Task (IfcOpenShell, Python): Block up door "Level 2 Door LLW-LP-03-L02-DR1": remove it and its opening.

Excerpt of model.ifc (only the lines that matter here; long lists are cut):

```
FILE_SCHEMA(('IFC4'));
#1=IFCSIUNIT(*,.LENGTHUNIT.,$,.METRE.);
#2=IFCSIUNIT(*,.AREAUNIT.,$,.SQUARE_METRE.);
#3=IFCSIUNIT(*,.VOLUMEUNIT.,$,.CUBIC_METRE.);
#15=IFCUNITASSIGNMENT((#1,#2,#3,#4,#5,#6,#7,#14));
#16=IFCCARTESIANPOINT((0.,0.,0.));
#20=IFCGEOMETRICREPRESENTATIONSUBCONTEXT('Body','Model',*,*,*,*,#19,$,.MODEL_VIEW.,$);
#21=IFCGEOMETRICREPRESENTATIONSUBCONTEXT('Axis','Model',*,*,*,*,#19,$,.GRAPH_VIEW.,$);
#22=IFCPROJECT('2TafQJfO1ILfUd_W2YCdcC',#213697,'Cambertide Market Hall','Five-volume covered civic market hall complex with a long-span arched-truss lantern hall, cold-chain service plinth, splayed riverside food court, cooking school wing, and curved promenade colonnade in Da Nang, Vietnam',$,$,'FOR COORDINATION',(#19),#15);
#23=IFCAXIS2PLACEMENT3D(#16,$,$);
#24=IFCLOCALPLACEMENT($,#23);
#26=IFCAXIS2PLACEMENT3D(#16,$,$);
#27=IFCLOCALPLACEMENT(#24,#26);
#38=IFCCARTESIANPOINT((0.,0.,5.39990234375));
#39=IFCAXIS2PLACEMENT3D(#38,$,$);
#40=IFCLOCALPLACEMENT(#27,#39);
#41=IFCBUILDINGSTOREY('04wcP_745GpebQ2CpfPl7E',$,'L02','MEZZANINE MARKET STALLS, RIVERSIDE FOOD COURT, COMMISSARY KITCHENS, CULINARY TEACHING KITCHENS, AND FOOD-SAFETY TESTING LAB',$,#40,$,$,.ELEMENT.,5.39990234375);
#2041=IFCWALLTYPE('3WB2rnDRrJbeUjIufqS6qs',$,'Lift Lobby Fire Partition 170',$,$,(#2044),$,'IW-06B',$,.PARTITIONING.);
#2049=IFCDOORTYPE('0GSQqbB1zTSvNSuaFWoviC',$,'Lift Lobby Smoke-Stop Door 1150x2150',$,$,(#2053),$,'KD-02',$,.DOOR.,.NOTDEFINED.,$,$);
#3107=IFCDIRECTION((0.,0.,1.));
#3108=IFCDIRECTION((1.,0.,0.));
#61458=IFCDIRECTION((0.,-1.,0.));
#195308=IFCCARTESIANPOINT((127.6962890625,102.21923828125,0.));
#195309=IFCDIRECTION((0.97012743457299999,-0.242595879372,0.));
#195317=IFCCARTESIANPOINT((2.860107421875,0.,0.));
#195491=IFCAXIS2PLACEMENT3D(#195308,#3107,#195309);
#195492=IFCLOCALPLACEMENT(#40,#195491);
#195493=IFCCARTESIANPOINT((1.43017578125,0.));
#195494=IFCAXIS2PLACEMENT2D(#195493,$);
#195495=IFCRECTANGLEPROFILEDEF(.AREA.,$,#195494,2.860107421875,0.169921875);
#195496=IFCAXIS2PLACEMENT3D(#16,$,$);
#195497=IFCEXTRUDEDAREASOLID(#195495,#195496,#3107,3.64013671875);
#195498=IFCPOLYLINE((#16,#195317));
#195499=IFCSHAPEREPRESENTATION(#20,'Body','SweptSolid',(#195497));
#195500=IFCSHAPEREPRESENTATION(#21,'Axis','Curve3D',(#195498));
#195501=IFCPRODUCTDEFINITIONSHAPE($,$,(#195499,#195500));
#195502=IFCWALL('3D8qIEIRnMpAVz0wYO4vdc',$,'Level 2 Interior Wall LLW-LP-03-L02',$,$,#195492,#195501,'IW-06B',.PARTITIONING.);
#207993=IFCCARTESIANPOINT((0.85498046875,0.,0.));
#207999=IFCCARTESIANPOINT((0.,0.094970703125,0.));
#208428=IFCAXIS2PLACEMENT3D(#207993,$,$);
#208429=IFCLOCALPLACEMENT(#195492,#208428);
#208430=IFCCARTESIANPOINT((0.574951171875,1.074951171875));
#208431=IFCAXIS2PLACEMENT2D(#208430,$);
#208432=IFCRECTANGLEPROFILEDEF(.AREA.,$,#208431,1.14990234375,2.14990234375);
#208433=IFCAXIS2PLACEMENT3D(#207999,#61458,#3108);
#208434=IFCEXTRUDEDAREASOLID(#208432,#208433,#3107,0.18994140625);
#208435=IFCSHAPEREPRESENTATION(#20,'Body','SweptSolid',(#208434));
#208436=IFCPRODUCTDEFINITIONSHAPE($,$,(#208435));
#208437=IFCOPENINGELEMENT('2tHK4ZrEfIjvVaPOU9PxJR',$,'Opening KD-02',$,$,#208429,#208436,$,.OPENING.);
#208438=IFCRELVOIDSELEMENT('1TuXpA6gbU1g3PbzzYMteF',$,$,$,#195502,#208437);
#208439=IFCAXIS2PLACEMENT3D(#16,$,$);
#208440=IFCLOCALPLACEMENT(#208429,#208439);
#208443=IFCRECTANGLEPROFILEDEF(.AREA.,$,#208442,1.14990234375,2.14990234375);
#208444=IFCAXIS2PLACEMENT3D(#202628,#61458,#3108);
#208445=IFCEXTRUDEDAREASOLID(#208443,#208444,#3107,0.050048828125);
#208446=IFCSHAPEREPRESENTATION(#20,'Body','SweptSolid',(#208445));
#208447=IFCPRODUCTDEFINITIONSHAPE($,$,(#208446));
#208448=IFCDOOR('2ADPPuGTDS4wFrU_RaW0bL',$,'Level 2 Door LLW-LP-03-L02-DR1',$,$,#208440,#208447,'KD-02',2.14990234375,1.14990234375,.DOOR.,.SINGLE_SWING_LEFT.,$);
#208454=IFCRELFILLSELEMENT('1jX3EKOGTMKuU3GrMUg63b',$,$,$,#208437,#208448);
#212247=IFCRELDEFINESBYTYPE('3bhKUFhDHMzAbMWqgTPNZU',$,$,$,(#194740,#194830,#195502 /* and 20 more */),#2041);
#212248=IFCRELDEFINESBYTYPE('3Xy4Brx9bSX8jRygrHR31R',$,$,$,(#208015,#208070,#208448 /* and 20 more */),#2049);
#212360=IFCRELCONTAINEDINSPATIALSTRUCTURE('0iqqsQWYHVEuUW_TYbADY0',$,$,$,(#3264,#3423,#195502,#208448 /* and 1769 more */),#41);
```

```python
import ifcopenshell
import ifcopenshell.api.feature
import ifcopenshell.api.root
import ifcopenshell.geom
import ifcopenshell.util.shape

model = ifcopenshell.open("model.ifc")
settings = ifcopenshell.geom.settings()


def volume(element):
    """Net volume in cubic metres, openings subtracted."""
    shape = ifcopenshell.geom.create_shape(settings, element)
    return ifcopenshell.util.shape.get_volume(shape.geometry)


door = model.by_id(208448)
opening = door.FillsVoids[0].RelatingOpeningElement
wall = opening.VoidsElements[0].RelatingBuildingElement
before = volume(wall)

ifcopenshell.api.root.remove_product(model, product=door)
ifcopenshell.api.feature.remove_feature(model, feature=opening)

after = volume(wall)

print(f"wall volume {before:.3f} -> {after:.3f} m3")

model.write("model_rev.ifc")
```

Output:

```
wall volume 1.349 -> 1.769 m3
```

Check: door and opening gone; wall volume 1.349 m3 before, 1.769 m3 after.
